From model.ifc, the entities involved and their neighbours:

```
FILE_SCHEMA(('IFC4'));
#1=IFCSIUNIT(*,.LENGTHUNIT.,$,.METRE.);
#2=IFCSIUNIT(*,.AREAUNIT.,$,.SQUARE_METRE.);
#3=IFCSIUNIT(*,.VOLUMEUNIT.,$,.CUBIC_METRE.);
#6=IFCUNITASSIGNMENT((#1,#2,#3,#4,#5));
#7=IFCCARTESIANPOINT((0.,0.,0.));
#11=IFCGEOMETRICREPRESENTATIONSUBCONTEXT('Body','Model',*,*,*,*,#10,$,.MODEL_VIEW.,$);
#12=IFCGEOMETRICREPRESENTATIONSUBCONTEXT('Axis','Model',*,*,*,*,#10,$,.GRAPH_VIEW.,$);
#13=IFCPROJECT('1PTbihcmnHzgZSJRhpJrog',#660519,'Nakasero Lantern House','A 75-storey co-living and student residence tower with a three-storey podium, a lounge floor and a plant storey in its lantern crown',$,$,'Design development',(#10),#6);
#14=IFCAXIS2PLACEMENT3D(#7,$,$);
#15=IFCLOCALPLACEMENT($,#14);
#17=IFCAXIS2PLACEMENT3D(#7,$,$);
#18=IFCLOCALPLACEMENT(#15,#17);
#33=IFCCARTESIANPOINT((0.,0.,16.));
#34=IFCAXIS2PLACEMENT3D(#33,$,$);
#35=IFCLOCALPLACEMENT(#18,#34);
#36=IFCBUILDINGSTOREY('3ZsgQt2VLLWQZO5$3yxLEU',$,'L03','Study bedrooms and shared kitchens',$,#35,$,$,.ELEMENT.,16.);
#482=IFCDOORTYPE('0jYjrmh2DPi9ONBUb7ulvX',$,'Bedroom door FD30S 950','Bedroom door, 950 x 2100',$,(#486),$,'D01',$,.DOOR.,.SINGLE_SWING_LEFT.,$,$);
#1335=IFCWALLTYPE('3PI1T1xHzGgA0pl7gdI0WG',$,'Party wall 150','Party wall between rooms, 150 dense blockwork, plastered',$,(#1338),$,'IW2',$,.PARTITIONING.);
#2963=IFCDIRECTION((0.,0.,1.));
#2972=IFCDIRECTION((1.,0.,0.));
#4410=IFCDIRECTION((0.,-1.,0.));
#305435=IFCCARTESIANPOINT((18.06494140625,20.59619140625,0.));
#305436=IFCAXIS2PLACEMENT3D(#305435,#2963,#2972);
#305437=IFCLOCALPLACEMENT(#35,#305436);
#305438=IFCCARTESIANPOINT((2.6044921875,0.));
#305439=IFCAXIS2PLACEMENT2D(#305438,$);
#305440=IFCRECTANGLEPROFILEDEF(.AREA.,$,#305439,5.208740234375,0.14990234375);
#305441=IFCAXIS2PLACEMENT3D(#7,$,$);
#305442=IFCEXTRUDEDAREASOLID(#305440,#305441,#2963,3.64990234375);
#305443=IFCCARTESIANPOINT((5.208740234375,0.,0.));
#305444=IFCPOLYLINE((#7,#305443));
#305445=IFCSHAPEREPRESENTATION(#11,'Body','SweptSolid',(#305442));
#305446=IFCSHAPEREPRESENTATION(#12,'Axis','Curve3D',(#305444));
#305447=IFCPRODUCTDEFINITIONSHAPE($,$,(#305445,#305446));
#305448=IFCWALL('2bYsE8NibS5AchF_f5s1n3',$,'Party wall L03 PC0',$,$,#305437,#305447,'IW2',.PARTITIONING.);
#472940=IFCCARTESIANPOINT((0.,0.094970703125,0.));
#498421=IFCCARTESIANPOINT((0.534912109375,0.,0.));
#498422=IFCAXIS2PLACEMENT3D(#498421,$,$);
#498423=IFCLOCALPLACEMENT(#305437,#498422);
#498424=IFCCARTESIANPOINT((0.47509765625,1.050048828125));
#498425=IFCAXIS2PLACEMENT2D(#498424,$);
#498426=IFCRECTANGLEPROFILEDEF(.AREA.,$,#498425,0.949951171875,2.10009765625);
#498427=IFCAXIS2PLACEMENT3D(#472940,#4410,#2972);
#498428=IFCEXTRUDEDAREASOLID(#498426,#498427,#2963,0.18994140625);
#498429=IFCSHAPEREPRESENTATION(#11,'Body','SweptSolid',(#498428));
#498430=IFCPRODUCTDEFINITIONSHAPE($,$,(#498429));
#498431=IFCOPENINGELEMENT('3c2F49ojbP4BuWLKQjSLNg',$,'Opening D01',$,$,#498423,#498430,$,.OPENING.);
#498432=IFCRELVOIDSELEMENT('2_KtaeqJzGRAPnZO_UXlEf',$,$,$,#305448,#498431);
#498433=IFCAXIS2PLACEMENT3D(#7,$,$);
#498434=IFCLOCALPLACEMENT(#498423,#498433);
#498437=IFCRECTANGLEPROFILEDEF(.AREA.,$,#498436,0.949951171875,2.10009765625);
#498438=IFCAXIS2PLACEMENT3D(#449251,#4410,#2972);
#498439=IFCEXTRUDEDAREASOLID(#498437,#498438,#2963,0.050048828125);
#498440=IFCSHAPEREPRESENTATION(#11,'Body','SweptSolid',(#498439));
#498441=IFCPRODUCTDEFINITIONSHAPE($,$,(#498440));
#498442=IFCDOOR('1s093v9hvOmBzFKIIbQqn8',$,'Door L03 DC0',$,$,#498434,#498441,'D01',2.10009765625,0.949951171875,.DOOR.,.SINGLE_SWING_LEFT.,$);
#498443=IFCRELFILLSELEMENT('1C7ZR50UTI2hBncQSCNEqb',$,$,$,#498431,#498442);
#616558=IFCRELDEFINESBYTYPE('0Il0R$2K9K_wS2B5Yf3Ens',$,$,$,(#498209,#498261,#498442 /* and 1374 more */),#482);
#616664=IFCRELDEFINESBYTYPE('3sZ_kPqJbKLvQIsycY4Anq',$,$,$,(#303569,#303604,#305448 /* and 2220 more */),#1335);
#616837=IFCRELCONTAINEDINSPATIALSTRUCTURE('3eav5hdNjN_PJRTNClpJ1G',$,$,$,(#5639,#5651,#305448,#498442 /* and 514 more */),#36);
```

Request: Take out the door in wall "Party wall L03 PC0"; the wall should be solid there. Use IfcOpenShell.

```python
import ifcopenshell
import ifcopenshell.api.feature
import ifcopenshell.api.root
import ifcopenshell.geom
import ifcopenshell.util.shape

model = ifcopenshell.open("model.ifc")
settings = ifcopenshell.geom.settings()


def volume(element):
    """Net volume in cubic metres, openings subtracted."""
    shape = ifcopenshell.geom.create_shape(settings, element)
    return ifcopenshell.util.shape.get_volume(shape.geometry)


door = model.by_id(498442)
opening = door.FillsVoids[0].RelatingOpeningElement
wall = opening.VoidsElements[0].RelatingBuildingElement
before = volume(wall)

ifcopenshell.api.root.remove_product(model, product=door)
ifcopenshell.api.feature.remove_feature(model, feature=opening)

after = volume(wall)

print(f"wall volume {before:.3f} -> {after:.3f} m3")

model.write("model-out.ifc")
```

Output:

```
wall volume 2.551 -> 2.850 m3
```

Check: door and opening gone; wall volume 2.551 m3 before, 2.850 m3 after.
